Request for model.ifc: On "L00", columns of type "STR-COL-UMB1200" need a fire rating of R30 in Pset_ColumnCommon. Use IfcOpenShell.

First a look at what the model holds.

```python
import ifcopenshell
import ifcopenshell.util.element

model = ifcopenshell.open("model.ifc")
print(model.schema)
storey = next(s for s in model.by_type("IfcBuildingStorey") if s.Name == "L00")
columns = [e for e in ifcopenshell.util.element.get_decomposition(storey) if e.is_a("IfcColumn")]
seen = {}
for e in columns:
    element_type = ifcopenshell.util.element.get_type(e)
    key = (element_type.Name if element_type != e and element_type else None, ifcopenshell.util.element.get_pset(e, "Pset_ColumnCommon", "FireRating"))
    seen[key] = seen.get(key, 0) + 1
for (name, value), count in sorted(seen.items(), key=str):
    print(count, "x", name, "|", value)
```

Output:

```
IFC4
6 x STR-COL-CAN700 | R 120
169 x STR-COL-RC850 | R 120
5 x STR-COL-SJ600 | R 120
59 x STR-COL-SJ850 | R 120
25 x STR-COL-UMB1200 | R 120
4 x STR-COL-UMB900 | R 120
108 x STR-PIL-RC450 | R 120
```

```python
import ifcopenshell
import ifcopenshell.api.pset
import ifcopenshell.util.element

model = ifcopenshell.open("model.ifc")

storey = next(s for s in model.by_type("IfcBuildingStorey") if s.Name == "L00")
columns = [e for e in ifcopenshell.util.element.get_decomposition(storey) if e.is_a("IfcColumn")]

count = 0
for e in columns:
    element_type = ifcopenshell.util.element.get_type(e)
    if element_type in (None, e) or element_type.Name != "STR-COL-UMB1200":
        continue
    # add_pset returns the element's existing set when there is one.
    pset = ifcopenshell.api.pset.add_pset(model, product=e, name="Pset_ColumnCommon")
    ifcopenshell.api.pset.edit_pset(model, pset=pset, properties={"FireRating": "R30"})
    count += 1

print(count, "columns updated")

model.write("model_rev.ifc")
```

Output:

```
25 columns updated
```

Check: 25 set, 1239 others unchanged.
